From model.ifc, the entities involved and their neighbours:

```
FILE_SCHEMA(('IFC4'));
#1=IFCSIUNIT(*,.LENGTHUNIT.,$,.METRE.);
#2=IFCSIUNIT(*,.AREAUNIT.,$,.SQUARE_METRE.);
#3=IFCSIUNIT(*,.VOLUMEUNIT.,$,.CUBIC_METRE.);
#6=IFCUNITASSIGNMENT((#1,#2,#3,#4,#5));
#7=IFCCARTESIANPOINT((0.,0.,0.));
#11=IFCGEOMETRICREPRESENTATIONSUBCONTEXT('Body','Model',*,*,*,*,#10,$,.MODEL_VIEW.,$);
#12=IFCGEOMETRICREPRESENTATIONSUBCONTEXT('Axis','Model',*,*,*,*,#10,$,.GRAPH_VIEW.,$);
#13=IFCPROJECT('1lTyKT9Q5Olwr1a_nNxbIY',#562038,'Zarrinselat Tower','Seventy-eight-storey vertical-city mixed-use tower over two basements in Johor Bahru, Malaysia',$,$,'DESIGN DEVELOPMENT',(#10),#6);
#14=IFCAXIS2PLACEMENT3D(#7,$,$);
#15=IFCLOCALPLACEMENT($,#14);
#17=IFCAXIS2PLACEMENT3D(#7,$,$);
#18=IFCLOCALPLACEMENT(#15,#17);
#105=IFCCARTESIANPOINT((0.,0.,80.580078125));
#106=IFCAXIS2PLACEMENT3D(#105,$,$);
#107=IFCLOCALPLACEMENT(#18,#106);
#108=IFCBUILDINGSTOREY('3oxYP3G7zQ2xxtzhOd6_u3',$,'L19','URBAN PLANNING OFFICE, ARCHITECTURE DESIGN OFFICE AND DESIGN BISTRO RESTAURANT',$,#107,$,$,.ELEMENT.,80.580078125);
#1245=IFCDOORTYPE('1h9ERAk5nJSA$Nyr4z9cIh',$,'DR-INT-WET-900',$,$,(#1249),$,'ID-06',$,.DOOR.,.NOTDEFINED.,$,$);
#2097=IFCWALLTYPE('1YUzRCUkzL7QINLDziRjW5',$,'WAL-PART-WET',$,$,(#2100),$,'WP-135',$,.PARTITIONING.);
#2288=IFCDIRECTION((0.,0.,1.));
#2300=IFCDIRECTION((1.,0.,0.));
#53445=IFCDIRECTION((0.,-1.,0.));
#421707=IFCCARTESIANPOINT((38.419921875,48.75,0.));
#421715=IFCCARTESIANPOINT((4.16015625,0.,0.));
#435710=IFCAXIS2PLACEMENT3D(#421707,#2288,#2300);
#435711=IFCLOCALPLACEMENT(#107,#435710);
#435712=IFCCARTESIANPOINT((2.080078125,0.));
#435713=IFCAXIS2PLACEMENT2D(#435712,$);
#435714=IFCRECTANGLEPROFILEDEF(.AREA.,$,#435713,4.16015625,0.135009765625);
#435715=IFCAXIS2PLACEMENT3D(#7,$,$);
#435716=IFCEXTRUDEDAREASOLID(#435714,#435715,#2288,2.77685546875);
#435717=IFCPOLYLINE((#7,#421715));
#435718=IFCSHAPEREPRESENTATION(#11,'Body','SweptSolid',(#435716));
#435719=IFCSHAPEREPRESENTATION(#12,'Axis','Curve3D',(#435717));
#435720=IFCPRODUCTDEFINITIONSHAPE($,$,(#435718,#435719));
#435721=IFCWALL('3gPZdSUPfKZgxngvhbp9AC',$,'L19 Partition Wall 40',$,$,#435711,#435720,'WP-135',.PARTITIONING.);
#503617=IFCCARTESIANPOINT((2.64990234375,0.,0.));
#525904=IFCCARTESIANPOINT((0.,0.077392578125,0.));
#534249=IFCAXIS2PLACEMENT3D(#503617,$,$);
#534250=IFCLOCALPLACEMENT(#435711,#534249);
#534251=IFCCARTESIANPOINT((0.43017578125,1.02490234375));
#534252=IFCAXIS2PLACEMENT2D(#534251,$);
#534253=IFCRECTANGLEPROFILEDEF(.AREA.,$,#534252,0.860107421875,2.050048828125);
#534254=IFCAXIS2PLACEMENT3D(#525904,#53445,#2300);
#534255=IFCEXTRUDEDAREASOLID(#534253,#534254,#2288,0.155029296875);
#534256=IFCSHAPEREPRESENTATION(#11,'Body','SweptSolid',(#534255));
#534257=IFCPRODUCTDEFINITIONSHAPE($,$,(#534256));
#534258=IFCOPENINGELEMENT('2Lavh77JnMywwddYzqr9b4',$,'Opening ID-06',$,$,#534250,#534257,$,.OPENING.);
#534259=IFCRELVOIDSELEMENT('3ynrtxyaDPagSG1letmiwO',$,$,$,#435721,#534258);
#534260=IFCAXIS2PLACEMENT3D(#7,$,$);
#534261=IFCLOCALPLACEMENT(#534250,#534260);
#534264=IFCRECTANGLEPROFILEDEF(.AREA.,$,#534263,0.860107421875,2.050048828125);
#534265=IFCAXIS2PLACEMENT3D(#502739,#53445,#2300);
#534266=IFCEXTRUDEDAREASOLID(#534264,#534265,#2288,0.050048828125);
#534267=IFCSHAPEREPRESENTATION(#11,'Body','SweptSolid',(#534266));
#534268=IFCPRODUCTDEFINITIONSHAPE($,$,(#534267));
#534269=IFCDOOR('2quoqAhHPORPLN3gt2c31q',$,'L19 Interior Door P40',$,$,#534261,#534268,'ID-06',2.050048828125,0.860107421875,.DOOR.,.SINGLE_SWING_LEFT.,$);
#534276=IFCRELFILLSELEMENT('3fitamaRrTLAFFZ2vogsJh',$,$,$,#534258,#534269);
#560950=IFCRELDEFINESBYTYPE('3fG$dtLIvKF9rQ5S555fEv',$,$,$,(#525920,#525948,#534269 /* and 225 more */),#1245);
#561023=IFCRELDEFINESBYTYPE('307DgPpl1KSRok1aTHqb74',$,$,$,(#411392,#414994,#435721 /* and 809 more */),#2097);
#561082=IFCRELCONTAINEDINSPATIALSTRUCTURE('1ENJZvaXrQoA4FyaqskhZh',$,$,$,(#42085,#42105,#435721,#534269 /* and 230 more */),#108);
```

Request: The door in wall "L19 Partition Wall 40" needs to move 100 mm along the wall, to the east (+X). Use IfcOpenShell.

```python
import ifcopenshell
import ifcopenshell.api.geometry
import ifcopenshell.util.placement

model = ifcopenshell.open("model.ifc")

door = model.by_guid("2quoqAhHPORPLN3gt2c31q")
opening = door.FillsVoids[0].RelatingOpeningElement
wall = opening.VoidsElements[0].RelatingBuildingElement

wall_matrix = ifcopenshell.util.placement.get_local_placement(wall.ObjectPlacement)
shift = wall_matrix[:3, 0] * 0.1
before = ifcopenshell.util.placement.get_local_placement(door.ObjectPlacement)[:3, 3].copy()

# The door is placed relative to its opening, so it follows when the opening moves.
matrix = ifcopenshell.util.placement.get_local_placement(opening.ObjectPlacement)
matrix[:3, 3] += shift
ifcopenshell.api.geometry.edit_object_placement(
    model, product=opening, matrix=matrix, is_si=False, should_transform_children=True
)

after = ifcopenshell.util.placement.get_local_placement(door.ObjectPlacement)[:3, 3]
print("door moved by", (after - before).round(3) + 0.0)

model.write("model_updated.ifc")
```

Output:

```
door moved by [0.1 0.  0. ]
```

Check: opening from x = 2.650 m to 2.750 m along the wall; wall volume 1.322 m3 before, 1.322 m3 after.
